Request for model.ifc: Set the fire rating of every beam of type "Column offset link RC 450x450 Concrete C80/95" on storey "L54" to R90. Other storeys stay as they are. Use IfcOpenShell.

First a look at what the model holds.

```python
import ifcopenshell
import ifcopenshell.util.element

model = ifcopenshell.open("model.ifc")
print(model.schema)
storey = next(s for s in model.by_type("IfcBuildingStorey") if s.Name == "L54")
beams = [e for e in ifcopenshell.util.element.get_decomposition(storey) if e.is_a("IfcBeam")]
seen = {}
for e in beams:
    element_type = ifcopenshell.util.element.get_type(e)
    key = (element_type.Name if element_type != e and element_type else None, ifcopenshell.util.element.get_pset(e, "Pset_BeamCommon", "FireRating"))
    seen[key] = seen.get(key, 0) + 1
for (name, value), count in sorted(seen.items(), key=str):
    print(count, "x", name, "|", value)
```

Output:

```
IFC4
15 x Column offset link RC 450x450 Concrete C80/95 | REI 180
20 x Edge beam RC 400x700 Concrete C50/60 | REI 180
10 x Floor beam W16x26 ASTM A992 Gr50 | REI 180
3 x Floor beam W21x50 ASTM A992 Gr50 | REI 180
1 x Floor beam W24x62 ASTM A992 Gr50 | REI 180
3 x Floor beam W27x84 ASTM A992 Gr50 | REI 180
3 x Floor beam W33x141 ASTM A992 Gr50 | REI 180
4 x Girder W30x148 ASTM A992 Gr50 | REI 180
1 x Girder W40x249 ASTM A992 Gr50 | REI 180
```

```python
import ifcopenshell
import ifcopenshell.api.pset
import ifcopenshell.util.element

model = ifcopenshell.open("model.ifc")

storey = next(s for s in model.by_type("IfcBuildingStorey") if s.Name == "L54")
beams = [e for e in ifcopenshell.util.element.get_decomposition(storey) if e.is_a("IfcBeam")]

count = 0
for e in beams:
    element_type = ifcopenshell.util.element.get_type(e)
    if element_type in (None, e) or element_type.Name != "Column offset link RC 450x450 Concrete C80/95":
        continue
    found = ifcopenshell.util.element.get_pset(e, "Pset_BeamCommon", should_inherit=False)
    if found:
        pset = model.by_id(found["id"])
        if len(ifcopenshell.util.element.get_elements_by_pset(pset)) > 1:
            pset = ifcopenshell.api.pset.unshare_pset(model, products=[e], pset=pset)[0]
    else:
        pset = ifcopenshell.api.pset.add_pset(model, product=e, name="Pset_BeamCommon")
    ifcopenshell.api.pset.edit_pset(model, pset=pset, properties={"FireRating": "R90"})
    count += 1

print(count, "beams updated")

model.write("model_v2.ifc")
```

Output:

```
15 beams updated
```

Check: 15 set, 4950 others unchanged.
